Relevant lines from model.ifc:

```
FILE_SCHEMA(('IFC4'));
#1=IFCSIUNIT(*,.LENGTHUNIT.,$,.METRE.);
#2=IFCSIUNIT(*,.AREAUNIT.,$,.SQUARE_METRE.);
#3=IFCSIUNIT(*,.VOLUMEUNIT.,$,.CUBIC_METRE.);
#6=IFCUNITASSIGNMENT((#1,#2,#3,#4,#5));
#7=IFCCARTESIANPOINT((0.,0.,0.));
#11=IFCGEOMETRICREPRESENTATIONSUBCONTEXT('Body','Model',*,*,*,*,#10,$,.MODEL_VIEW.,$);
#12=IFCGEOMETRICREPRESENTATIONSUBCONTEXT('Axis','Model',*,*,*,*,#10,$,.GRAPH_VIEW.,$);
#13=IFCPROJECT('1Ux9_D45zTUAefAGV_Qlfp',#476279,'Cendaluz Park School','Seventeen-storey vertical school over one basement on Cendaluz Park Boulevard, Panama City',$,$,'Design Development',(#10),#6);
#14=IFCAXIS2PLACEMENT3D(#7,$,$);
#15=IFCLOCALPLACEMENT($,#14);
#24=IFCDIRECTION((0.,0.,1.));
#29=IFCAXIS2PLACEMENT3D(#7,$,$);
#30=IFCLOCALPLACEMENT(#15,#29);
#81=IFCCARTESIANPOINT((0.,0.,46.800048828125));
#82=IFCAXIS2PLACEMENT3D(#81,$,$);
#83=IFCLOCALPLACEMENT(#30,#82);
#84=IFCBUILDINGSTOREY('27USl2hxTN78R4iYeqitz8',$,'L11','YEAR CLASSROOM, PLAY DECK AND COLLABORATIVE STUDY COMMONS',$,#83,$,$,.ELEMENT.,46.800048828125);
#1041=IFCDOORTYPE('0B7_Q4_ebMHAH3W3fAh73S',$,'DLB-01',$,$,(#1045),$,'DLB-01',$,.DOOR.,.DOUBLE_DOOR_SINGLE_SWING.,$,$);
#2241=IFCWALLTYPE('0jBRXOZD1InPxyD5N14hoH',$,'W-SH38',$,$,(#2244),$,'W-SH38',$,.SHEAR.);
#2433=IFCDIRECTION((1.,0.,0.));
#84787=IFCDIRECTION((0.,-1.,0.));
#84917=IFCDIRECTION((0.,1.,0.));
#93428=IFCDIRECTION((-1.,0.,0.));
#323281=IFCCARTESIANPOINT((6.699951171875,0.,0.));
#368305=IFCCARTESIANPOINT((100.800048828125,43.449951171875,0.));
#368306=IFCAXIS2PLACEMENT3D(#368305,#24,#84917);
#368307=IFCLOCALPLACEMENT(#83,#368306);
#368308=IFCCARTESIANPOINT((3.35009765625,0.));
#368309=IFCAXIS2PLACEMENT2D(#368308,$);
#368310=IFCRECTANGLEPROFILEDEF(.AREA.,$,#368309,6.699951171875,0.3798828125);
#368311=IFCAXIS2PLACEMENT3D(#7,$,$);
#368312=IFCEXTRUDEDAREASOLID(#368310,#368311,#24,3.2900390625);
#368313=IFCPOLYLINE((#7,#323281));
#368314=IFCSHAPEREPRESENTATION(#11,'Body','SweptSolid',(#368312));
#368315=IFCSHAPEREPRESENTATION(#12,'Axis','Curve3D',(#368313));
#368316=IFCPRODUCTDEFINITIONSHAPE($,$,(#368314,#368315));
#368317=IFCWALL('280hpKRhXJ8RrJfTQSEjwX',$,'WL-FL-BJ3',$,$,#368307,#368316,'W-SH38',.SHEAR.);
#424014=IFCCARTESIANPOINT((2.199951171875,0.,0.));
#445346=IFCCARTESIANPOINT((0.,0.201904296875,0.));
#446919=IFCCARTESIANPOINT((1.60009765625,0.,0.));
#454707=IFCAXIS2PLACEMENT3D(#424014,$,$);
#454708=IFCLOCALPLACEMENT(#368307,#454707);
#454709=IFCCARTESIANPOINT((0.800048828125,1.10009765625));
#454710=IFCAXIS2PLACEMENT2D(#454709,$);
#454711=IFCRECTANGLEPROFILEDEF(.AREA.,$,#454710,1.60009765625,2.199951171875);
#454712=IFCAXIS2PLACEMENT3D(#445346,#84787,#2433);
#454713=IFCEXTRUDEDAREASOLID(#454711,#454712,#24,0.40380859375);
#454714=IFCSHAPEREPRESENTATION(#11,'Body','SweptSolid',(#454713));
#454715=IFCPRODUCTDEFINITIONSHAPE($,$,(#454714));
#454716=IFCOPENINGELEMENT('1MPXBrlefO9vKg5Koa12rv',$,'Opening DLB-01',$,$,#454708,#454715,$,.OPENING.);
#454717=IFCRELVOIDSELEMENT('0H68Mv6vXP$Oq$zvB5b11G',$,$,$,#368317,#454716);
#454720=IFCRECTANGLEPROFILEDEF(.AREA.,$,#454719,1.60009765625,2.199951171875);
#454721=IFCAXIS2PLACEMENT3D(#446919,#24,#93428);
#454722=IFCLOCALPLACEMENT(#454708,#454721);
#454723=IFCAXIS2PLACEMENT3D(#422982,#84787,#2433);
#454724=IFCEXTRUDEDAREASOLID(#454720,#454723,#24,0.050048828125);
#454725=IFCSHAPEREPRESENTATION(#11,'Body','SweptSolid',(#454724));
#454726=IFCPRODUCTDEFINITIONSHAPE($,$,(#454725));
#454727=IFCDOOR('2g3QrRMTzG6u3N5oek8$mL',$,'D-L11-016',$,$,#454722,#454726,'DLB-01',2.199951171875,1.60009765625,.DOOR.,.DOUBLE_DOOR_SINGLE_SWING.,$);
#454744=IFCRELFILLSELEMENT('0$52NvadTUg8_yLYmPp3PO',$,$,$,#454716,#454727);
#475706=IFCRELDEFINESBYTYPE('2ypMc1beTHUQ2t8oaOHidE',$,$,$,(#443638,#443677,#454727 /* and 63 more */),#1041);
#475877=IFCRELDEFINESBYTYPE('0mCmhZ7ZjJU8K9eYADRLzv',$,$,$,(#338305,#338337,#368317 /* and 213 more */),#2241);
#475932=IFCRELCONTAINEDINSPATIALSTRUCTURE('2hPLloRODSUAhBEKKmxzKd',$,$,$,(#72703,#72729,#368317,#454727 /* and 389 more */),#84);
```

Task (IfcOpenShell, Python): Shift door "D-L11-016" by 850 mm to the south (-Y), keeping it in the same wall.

```python
import ifcopenshell
import ifcopenshell.api.geometry
import ifcopenshell.util.placement

model = ifcopenshell.open("model.ifc")

door = model.by_id(454727)
opening = door.FillsVoids[0].RelatingOpeningElement
wall = opening.VoidsElements[0].RelatingBuildingElement

wall_matrix = ifcopenshell.util.placement.get_local_placement(wall.ObjectPlacement)
shift = wall_matrix[:3, 0] * -0.85
before = ifcopenshell.util.placement.get_local_placement(door.ObjectPlacement)[:3, 3].copy()

# The door is placed relative to its opening, so it follows when the opening moves.
matrix = ifcopenshell.util.placement.get_local_placement(opening.ObjectPlacement)
matrix[:3, 3] += shift
ifcopenshell.api.geometry.edit_object_placement(
    model, product=opening, matrix=matrix, is_si=False, should_transform_children=True
)

after = ifcopenshell.util.placement.get_local_placement(door.ObjectPlacement)[:3, 3]
print("door moved by", (after - before).round(3) + 0.0)

model.write("model-out.ifc")
```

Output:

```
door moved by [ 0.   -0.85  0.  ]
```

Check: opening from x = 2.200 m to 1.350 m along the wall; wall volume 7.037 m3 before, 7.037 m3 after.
